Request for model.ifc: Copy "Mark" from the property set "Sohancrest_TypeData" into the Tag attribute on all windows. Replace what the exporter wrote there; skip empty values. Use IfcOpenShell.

First a look at what the model holds.

```python
import ifcopenshell
import ifcopenshell.util.element

model = ifcopenshell.open("model.ifc")
print(model.schema)
windows = model.by_type("IfcWindow")
print(len(windows), "windows")
for e in windows[:8]:
    source = ifcopenshell.util.element.get_pset(e, "Sohancrest_TypeData", "Mark")
    target = e.Tag
    print(e.id(), repr(source), repr(target), sep=" | ")
```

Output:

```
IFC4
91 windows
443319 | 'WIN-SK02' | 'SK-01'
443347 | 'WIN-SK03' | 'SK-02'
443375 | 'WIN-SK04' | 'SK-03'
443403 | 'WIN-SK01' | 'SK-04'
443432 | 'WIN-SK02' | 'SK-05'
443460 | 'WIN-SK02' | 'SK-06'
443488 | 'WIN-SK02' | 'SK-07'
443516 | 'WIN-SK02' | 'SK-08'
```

```python
import ifcopenshell
import ifcopenshell.util.element

model = ifcopenshell.open("model.ifc")

count = 0
for e in model.by_type("IfcWindow"):
    value = ifcopenshell.util.element.get_pset(e, "Sohancrest_TypeData", "Mark")
    current = e.Tag
    if not value or not value.strip() or current == value:
        continue
    e.Tag = value
    count += 1

print(count, "windows updated")

model.write("model_updated.ifc")
```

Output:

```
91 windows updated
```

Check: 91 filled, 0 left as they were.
